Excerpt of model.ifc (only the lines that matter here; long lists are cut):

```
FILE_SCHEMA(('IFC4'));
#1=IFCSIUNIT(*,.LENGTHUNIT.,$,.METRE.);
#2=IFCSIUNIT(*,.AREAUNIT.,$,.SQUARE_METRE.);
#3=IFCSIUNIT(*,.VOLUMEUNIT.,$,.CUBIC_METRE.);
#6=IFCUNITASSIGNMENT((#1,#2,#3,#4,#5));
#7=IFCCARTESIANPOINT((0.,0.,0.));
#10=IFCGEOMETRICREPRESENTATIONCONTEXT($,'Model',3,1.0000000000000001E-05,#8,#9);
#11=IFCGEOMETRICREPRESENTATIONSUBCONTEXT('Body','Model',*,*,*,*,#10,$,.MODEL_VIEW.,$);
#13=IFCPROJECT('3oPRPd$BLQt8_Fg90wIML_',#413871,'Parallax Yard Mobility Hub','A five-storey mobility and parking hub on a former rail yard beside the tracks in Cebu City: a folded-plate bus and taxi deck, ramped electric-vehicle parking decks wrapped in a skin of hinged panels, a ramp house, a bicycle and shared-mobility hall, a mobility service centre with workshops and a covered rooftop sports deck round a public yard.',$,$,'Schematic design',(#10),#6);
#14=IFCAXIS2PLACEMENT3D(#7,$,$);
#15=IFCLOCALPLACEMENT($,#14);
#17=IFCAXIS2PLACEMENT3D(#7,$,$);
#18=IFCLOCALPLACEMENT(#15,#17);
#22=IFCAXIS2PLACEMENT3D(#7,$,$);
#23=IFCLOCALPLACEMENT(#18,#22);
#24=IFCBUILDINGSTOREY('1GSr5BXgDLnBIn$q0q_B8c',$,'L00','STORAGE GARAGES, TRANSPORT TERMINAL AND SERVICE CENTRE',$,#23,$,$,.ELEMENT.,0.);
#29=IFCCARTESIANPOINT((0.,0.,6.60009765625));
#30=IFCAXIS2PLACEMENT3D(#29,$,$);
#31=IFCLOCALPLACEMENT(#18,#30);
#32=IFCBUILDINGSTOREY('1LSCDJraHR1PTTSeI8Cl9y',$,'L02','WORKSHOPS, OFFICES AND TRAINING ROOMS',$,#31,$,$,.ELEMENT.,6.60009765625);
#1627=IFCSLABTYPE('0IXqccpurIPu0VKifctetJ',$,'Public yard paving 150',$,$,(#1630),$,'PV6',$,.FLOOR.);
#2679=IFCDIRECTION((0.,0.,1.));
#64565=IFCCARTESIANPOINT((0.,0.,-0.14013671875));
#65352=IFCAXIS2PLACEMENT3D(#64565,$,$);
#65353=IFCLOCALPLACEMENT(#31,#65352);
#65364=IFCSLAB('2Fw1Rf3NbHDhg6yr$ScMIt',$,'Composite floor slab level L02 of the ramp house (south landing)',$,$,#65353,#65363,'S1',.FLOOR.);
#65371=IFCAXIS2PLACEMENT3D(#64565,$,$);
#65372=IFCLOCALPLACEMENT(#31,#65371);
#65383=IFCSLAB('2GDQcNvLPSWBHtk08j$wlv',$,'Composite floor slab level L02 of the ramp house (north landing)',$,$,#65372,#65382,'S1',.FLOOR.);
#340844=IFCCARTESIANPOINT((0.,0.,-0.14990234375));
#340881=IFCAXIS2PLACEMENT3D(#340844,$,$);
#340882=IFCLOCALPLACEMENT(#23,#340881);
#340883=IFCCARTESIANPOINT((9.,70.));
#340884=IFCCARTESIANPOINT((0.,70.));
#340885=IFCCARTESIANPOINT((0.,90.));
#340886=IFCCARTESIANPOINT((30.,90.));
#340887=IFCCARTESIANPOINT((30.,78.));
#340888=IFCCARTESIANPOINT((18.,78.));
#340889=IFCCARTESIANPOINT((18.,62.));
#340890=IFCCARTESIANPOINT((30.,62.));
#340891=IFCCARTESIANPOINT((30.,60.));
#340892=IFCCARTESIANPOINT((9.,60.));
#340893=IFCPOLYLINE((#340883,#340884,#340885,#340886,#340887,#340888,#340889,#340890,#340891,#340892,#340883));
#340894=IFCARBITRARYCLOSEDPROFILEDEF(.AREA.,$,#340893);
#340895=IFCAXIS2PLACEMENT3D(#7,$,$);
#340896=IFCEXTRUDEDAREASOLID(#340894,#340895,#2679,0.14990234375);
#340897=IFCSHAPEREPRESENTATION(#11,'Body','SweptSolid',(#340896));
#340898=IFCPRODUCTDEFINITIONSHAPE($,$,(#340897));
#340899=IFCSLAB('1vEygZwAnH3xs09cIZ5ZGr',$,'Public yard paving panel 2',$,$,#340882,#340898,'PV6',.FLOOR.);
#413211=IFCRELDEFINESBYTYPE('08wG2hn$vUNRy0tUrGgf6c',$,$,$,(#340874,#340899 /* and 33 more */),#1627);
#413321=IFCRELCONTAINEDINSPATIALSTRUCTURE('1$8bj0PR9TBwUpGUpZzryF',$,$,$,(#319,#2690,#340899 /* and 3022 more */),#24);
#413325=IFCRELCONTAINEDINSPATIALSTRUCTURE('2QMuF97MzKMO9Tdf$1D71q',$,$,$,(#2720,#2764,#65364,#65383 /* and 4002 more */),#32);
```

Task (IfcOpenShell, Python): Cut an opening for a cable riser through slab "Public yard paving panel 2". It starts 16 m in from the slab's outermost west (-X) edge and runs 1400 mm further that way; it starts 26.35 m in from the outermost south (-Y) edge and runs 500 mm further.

```python
import numpy as np
import ifcopenshell
import ifcopenshell.api.feature
import ifcopenshell.api.geometry
import ifcopenshell.api.root
import ifcopenshell.geom
import ifcopenshell.util.placement
import ifcopenshell.util.representation
import ifcopenshell.util.shape
import ifcopenshell.util.unit

model = ifcopenshell.open("model.ifc")
unit_scale = ifcopenshell.util.unit.calculate_unit_scale(model)
settings = ifcopenshell.geom.settings()


def volume(element):
    """Net volume in cubic metres, openings subtracted."""
    shape = ifcopenshell.geom.create_shape(settings, element)
    return ifcopenshell.util.shape.get_volume(shape.geometry)


slab = model.by_id(340899)
before = volume(slab)

# Extent in the slab's own axes, in metres. The edges named are its -X and -Y sides.
slab_shape = ifcopenshell.geom.create_shape(settings, slab)
vertices = ifcopenshell.util.shape.get_vertices(slab_shape.geometry)
x_min, y_min, bottom = vertices.min(axis=0)
top = vertices[:, 2].max()

opening = ifcopenshell.api.root.create_entity(model, ifc_class="IfcOpeningElement", name="Cable riser opening", predefined_type="OPENING")
context = ifcopenshell.util.representation.get_context(model, "Model", "Body", "MODEL_VIEW")
width, depth = 1.4, 0.5
outline = [(0.0, 0.0), (width, 0.0), (width, depth), (0.0, depth), (0.0, 0.0)]
# Overshoot both faces by 50 mm so the cut is clean.
shape = ifcopenshell.api.geometry.add_slab_representation(
    model, context=context, depth=top - bottom + 0.1, polyline=outline
)
ifcopenshell.api.geometry.assign_representation(model, product=opening, representation=shape)

matrix = ifcopenshell.util.placement.get_local_placement(slab.ObjectPlacement)
matrix[:, 3] = matrix @ np.append(np.array([x_min + 16, y_min + 26.35, bottom - 0.05]) / unit_scale, 1.0)
ifcopenshell.api.geometry.edit_object_placement(model, product=opening, matrix=matrix, is_si=False)
ifcopenshell.api.feature.add_feature(model, feature=opening, element=slab)

after = volume(slab)

print(f"slab volume {before:.3f} -> {after:.3f} m3")

model.write("model-out.ifc")
```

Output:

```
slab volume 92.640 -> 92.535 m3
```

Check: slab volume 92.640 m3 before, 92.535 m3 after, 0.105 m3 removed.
